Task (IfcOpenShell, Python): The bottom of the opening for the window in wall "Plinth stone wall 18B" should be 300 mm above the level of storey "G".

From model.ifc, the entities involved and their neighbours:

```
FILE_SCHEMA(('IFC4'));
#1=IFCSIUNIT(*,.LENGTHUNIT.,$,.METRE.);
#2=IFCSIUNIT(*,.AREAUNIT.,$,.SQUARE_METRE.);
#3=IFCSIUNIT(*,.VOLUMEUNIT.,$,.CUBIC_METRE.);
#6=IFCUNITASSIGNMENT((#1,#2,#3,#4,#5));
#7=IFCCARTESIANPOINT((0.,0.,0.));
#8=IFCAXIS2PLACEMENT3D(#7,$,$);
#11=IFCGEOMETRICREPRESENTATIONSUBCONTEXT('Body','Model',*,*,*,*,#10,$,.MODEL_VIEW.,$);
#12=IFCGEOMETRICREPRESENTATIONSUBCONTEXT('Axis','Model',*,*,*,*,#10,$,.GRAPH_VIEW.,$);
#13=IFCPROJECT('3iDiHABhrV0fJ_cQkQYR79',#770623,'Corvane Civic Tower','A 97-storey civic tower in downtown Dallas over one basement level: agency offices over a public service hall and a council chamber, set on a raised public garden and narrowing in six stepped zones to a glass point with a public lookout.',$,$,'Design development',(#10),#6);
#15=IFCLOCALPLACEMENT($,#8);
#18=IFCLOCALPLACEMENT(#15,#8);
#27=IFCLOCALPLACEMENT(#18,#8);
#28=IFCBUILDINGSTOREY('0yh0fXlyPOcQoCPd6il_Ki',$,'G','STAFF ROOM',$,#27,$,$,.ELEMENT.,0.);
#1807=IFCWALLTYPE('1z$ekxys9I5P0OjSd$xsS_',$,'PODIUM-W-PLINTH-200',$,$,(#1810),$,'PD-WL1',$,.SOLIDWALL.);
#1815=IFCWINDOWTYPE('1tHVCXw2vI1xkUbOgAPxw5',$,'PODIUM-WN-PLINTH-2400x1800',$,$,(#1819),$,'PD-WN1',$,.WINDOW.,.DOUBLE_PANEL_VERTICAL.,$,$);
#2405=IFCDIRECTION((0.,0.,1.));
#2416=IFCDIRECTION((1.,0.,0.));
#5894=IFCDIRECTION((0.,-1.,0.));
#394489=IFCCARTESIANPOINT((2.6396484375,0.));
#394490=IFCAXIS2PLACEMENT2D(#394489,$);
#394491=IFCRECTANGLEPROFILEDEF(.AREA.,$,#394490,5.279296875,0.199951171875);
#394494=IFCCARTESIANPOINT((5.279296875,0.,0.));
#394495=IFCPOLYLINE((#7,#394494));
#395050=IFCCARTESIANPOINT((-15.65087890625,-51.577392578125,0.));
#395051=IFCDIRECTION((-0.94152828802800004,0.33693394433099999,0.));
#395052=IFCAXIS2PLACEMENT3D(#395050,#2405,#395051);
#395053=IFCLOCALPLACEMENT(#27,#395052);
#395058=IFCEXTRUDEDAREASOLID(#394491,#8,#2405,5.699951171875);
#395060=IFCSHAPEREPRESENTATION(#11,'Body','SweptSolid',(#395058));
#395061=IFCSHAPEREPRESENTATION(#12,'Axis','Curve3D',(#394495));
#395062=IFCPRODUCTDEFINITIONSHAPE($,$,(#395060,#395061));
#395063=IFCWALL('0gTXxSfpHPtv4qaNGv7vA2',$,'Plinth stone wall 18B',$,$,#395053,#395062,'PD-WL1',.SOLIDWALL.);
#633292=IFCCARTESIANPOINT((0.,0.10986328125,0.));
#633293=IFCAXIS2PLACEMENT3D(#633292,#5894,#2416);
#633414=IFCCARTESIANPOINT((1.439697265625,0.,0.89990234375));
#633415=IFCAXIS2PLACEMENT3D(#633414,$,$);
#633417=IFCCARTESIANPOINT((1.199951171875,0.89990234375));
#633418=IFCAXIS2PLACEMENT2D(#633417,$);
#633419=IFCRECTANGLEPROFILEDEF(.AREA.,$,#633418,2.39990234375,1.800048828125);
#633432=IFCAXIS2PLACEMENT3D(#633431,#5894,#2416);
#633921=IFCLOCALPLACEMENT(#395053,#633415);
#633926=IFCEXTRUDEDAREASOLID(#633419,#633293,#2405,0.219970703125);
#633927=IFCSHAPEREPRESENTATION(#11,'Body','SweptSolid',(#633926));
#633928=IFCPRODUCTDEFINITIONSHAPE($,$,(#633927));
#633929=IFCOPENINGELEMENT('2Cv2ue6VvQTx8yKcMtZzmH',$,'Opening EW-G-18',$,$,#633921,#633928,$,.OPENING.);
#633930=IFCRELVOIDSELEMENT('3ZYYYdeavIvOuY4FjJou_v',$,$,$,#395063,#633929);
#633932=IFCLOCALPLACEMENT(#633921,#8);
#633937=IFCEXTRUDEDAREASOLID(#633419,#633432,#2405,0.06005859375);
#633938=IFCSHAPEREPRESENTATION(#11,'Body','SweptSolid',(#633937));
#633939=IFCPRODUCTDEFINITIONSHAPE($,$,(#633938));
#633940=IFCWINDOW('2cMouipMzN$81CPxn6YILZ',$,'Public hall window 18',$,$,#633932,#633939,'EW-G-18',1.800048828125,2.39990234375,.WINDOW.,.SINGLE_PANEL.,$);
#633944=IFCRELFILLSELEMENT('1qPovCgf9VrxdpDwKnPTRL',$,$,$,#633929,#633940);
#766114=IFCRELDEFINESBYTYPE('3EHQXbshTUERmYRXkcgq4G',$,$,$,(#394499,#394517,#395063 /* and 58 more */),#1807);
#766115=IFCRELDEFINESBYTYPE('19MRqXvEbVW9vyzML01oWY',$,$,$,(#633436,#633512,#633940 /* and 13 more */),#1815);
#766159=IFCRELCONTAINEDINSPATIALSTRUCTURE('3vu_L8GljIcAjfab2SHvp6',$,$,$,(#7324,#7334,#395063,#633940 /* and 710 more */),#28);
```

```python
import numpy as np
import ifcopenshell
import ifcopenshell.api.geometry
import ifcopenshell.geom
import ifcopenshell.util.element
import ifcopenshell.util.placement
import ifcopenshell.util.shape
import ifcopenshell.util.unit

model = ifcopenshell.open("model.ifc")
unit_scale = ifcopenshell.util.unit.calculate_unit_scale(model)

window = model.by_guid("2cMouipMzN$81CPxn6YILZ")
opening = window.FillsVoids[0].RelatingOpeningElement
storey = ifcopenshell.util.element.get_container(window, ifc_class="IfcBuildingStorey")
level = ifcopenshell.util.placement.get_local_placement(storey.ObjectPlacement)[2, 3]

# The opening's origin need not be at the sill, so measure its lowest point.
shape = ifcopenshell.geom.create_shape(ifcopenshell.geom.settings(), opening)
bottom = ifcopenshell.util.shape.get_shape_bottom_elevation(shape, shape.geometry) / unit_scale
dz = level + 0.3 / unit_scale - bottom

shift = np.array([0.0, 0.0, dz])
# The window is placed relative to its opening, so it follows when the opening moves.
matrix = ifcopenshell.util.placement.get_local_placement(opening.ObjectPlacement)
matrix[:3, 3] += shift
ifcopenshell.api.geometry.edit_object_placement(
    model, product=opening, matrix=matrix, is_si=False, should_transform_children=True
)

print(f"moved by {dz * unit_scale:+.3f} m")

model.write("model_updated.ifc")
```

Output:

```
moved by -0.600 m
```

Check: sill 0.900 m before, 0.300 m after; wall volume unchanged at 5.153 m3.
